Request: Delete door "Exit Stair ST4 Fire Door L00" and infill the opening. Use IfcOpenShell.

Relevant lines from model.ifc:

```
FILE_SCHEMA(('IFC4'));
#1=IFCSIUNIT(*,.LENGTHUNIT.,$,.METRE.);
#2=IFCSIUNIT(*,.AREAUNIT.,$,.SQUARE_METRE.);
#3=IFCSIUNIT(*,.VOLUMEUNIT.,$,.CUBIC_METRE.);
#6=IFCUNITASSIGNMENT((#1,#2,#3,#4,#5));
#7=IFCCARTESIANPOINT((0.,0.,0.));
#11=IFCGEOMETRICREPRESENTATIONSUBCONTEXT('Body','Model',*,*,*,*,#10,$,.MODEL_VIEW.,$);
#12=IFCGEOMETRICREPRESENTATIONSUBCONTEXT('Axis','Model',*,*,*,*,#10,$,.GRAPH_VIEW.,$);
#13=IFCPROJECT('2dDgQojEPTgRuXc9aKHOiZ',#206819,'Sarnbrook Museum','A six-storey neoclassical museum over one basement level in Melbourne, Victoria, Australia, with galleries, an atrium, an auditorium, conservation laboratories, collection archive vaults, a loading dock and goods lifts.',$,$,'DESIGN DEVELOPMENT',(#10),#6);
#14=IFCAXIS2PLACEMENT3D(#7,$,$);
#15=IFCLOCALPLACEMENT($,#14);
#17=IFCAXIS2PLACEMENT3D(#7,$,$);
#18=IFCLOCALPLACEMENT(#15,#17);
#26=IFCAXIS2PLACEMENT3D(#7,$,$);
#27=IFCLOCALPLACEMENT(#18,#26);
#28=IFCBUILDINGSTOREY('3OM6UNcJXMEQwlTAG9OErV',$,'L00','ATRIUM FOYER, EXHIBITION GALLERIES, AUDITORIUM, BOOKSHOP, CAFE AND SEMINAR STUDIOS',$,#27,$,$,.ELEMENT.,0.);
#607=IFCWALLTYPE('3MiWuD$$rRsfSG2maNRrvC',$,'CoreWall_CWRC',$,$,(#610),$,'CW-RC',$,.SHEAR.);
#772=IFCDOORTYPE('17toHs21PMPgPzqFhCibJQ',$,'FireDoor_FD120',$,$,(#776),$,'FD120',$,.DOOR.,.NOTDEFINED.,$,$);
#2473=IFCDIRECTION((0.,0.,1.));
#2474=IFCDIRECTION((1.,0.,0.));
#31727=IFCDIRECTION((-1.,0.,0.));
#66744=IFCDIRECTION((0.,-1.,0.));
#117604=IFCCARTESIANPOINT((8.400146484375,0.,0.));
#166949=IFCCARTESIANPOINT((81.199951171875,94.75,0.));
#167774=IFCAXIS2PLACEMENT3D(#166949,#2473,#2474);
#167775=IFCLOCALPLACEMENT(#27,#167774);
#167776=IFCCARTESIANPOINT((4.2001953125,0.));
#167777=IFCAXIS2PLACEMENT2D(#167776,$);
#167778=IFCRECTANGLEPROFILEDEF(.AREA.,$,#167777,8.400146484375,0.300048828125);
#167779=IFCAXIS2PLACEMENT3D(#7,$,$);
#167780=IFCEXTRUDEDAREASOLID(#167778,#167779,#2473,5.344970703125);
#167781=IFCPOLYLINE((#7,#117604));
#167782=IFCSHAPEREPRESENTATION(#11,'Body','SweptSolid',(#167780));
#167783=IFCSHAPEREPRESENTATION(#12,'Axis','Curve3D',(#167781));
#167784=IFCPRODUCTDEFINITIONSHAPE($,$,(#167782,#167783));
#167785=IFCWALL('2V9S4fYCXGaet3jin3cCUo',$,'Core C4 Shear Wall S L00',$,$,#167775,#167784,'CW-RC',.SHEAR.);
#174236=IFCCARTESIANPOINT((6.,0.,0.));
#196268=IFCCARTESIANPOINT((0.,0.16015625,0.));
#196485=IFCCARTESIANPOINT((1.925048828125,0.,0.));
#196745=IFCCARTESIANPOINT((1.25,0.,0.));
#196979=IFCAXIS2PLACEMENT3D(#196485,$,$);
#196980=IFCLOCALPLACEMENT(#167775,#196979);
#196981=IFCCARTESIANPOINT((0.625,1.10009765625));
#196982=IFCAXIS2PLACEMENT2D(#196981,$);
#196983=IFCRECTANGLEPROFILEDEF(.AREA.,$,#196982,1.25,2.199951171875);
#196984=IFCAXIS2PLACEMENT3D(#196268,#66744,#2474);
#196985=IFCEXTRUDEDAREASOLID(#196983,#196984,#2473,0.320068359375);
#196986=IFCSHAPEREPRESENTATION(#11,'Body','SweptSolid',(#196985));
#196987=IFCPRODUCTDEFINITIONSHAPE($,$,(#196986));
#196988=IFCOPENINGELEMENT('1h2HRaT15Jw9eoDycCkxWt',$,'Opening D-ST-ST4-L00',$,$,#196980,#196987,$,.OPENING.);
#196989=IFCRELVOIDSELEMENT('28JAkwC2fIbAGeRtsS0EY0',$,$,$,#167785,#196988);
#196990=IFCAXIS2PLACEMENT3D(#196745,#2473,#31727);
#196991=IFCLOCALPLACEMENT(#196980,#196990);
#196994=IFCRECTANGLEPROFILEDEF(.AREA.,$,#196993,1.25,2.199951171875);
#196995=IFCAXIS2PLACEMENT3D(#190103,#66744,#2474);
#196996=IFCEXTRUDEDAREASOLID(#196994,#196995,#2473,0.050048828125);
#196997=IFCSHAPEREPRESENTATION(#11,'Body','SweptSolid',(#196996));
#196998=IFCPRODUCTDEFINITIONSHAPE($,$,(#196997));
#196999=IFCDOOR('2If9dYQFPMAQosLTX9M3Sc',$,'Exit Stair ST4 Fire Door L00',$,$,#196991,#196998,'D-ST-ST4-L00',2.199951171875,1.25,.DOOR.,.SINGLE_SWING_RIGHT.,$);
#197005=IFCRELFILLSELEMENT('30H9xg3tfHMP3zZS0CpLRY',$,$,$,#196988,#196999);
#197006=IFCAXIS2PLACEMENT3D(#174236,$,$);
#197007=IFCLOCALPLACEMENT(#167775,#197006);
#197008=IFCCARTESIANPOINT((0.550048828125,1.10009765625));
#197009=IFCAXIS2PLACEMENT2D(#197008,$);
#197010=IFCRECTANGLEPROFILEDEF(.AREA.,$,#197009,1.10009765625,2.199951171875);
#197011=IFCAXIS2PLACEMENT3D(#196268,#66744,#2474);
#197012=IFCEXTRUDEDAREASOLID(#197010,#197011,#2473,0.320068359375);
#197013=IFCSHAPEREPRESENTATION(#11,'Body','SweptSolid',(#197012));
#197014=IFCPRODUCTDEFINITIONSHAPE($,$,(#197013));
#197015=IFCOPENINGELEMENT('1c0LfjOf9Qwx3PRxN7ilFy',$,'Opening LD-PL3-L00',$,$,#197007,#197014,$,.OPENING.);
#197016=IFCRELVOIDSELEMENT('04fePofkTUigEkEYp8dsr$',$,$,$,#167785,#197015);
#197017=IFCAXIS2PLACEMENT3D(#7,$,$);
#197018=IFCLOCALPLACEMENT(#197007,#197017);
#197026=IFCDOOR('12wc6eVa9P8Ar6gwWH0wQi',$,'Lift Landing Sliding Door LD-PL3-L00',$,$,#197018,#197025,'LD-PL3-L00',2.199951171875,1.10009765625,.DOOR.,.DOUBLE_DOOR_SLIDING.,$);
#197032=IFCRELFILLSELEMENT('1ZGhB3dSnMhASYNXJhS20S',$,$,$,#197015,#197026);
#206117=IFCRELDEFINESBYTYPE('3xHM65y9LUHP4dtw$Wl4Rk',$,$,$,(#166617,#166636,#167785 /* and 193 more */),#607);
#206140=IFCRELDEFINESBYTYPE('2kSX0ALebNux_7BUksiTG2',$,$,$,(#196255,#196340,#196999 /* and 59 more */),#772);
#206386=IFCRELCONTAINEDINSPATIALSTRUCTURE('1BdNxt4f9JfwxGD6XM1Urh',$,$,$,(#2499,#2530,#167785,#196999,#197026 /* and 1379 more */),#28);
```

```python
import ifcopenshell
import ifcopenshell.api.feature
import ifcopenshell.api.root
import ifcopenshell.geom
import ifcopenshell.util.shape

model = ifcopenshell.open("model.ifc")
settings = ifcopenshell.geom.settings()


def volume(element):
    """Net volume in cubic metres, openings subtracted."""
    shape = ifcopenshell.geom.create_shape(settings, element)
    return ifcopenshell.util.shape.get_volume(shape.geometry)


door = model.by_guid("2If9dYQFPMAQosLTX9M3Sc")
opening = door.FillsVoids[0].RelatingOpeningElement
wall = opening.VoidsElements[0].RelatingBuildingElement
before = volume(wall)

ifcopenshell.api.root.remove_product(model, product=door)
ifcopenshell.api.feature.remove_feature(model, feature=opening)

after = volume(wall)

print(f"wall volume {before:.3f} -> {after:.3f} m3")

model.write("model_updated.ifc")
```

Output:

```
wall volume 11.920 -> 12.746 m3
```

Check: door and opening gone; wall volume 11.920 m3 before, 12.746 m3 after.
